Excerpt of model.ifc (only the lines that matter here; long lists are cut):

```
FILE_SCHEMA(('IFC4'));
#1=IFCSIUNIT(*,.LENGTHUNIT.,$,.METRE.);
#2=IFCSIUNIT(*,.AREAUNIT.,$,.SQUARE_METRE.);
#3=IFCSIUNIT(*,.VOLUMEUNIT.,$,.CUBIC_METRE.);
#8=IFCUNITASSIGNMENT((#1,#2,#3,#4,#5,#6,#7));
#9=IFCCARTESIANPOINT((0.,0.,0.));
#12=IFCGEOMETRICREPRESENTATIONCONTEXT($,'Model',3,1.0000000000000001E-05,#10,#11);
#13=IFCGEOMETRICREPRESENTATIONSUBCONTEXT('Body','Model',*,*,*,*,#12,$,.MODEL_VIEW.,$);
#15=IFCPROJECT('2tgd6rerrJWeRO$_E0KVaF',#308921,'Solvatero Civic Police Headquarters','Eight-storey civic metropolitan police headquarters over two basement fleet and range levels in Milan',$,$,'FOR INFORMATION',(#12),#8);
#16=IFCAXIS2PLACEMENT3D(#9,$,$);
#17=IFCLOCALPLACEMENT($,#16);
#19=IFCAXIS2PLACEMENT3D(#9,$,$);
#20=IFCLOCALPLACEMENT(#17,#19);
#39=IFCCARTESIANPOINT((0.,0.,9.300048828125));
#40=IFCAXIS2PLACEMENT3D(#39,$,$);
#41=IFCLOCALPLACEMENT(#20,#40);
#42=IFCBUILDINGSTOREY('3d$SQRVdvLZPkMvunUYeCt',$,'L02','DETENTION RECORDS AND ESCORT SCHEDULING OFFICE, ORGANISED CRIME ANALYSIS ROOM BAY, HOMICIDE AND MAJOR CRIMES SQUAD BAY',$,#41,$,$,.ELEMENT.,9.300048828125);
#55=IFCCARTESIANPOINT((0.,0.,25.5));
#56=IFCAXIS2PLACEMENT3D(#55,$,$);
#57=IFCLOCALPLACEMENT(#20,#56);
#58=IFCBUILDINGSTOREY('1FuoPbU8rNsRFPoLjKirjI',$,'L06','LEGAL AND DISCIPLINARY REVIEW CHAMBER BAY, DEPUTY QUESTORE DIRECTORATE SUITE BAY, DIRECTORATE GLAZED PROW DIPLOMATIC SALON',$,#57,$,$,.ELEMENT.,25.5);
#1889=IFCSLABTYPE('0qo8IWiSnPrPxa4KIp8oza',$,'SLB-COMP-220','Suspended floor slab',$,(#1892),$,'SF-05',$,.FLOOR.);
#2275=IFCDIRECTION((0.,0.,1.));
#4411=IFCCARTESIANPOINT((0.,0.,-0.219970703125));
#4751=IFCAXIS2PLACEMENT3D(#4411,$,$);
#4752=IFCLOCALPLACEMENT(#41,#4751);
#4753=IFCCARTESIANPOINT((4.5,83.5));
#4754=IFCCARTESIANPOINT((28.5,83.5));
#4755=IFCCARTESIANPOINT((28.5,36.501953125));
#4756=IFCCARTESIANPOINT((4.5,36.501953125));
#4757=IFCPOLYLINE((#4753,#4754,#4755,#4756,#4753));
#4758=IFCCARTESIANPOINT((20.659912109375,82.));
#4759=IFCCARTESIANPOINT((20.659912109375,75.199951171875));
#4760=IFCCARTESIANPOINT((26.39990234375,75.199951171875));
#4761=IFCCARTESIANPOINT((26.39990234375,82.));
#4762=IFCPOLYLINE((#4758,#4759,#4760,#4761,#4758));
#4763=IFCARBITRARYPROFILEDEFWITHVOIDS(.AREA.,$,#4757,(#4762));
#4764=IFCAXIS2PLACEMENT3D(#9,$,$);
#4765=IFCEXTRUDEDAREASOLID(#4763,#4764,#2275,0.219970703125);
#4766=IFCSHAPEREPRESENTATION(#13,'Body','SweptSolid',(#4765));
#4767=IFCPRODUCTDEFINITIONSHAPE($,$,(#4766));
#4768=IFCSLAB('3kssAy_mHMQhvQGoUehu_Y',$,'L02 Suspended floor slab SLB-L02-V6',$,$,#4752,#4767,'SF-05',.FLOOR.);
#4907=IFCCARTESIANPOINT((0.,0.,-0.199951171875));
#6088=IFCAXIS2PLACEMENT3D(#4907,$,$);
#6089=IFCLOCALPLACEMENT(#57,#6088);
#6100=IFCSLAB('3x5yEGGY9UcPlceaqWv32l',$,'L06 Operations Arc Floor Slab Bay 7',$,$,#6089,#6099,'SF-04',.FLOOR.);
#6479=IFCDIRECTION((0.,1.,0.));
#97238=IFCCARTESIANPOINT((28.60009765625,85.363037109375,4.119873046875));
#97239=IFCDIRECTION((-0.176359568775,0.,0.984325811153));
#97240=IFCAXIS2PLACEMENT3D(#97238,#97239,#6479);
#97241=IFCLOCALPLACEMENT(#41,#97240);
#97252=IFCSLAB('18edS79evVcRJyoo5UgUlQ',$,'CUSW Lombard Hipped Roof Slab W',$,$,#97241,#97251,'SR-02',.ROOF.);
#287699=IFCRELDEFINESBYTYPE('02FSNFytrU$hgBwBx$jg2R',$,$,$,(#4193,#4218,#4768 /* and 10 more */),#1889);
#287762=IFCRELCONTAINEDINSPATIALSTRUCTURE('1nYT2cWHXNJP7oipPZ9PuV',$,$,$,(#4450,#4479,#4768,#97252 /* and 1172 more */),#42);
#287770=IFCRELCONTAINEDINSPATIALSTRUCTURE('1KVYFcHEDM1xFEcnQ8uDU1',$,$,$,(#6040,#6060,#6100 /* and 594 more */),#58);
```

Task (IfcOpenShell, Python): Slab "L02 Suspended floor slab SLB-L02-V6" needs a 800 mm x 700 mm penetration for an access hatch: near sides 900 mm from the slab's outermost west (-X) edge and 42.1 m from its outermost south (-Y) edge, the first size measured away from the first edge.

```python
import numpy as np
import ifcopenshell
import ifcopenshell.api.feature
import ifcopenshell.api.geometry
import ifcopenshell.api.root
import ifcopenshell.geom
import ifcopenshell.util.placement
import ifcopenshell.util.representation
import ifcopenshell.util.shape
import ifcopenshell.util.unit

model = ifcopenshell.open("model.ifc")
unit_scale = ifcopenshell.util.unit.calculate_unit_scale(model)
settings = ifcopenshell.geom.settings()


def volume(element):
    """Net volume in cubic metres, openings subtracted."""
    shape = ifcopenshell.geom.create_shape(settings, element)
    return ifcopenshell.util.shape.get_volume(shape.geometry)


slab = model.by_id(4768)
before = volume(slab)

# Extent in the slab's own axes, in metres. The edges named are its -X and -Y sides.
slab_shape = ifcopenshell.geom.create_shape(settings, slab)
vertices = ifcopenshell.util.shape.get_vertices(slab_shape.geometry)
x_min, y_min, bottom = vertices.min(axis=0)
top = vertices[:, 2].max()

opening = ifcopenshell.api.root.create_entity(model, ifc_class="IfcOpeningElement", name="Access hatch opening", predefined_type="OPENING")
context = ifcopenshell.util.representation.get_context(model, "Model", "Body", "MODEL_VIEW")
width, depth = 0.8, 0.7
outline = [(0.0, 0.0), (width, 0.0), (width, depth), (0.0, depth), (0.0, 0.0)]
# Overshoot both faces by 50 mm so the cut is clean.
shape = ifcopenshell.api.geometry.add_slab_representation(
    model, context=context, depth=top - bottom + 0.1, polyline=outline
)
ifcopenshell.api.geometry.assign_representation(model, product=opening, representation=shape)

matrix = ifcopenshell.util.placement.get_local_placement(slab.ObjectPlacement)
matrix[:, 3] = matrix @ np.append(np.array([x_min + 0.9, y_min + 42.1, bottom - 0.05]) / unit_scale, 1.0)
ifcopenshell.api.geometry.edit_object_placement(model, product=opening, matrix=matrix, is_si=False)
ifcopenshell.api.feature.add_feature(model, feature=opening, element=slab)

after = volume(slab)

print(f"slab volume {before:.3f} -> {after:.3f} m3")

model.write("model_v2.ifc")
```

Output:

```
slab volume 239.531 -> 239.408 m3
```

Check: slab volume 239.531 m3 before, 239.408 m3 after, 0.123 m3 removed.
